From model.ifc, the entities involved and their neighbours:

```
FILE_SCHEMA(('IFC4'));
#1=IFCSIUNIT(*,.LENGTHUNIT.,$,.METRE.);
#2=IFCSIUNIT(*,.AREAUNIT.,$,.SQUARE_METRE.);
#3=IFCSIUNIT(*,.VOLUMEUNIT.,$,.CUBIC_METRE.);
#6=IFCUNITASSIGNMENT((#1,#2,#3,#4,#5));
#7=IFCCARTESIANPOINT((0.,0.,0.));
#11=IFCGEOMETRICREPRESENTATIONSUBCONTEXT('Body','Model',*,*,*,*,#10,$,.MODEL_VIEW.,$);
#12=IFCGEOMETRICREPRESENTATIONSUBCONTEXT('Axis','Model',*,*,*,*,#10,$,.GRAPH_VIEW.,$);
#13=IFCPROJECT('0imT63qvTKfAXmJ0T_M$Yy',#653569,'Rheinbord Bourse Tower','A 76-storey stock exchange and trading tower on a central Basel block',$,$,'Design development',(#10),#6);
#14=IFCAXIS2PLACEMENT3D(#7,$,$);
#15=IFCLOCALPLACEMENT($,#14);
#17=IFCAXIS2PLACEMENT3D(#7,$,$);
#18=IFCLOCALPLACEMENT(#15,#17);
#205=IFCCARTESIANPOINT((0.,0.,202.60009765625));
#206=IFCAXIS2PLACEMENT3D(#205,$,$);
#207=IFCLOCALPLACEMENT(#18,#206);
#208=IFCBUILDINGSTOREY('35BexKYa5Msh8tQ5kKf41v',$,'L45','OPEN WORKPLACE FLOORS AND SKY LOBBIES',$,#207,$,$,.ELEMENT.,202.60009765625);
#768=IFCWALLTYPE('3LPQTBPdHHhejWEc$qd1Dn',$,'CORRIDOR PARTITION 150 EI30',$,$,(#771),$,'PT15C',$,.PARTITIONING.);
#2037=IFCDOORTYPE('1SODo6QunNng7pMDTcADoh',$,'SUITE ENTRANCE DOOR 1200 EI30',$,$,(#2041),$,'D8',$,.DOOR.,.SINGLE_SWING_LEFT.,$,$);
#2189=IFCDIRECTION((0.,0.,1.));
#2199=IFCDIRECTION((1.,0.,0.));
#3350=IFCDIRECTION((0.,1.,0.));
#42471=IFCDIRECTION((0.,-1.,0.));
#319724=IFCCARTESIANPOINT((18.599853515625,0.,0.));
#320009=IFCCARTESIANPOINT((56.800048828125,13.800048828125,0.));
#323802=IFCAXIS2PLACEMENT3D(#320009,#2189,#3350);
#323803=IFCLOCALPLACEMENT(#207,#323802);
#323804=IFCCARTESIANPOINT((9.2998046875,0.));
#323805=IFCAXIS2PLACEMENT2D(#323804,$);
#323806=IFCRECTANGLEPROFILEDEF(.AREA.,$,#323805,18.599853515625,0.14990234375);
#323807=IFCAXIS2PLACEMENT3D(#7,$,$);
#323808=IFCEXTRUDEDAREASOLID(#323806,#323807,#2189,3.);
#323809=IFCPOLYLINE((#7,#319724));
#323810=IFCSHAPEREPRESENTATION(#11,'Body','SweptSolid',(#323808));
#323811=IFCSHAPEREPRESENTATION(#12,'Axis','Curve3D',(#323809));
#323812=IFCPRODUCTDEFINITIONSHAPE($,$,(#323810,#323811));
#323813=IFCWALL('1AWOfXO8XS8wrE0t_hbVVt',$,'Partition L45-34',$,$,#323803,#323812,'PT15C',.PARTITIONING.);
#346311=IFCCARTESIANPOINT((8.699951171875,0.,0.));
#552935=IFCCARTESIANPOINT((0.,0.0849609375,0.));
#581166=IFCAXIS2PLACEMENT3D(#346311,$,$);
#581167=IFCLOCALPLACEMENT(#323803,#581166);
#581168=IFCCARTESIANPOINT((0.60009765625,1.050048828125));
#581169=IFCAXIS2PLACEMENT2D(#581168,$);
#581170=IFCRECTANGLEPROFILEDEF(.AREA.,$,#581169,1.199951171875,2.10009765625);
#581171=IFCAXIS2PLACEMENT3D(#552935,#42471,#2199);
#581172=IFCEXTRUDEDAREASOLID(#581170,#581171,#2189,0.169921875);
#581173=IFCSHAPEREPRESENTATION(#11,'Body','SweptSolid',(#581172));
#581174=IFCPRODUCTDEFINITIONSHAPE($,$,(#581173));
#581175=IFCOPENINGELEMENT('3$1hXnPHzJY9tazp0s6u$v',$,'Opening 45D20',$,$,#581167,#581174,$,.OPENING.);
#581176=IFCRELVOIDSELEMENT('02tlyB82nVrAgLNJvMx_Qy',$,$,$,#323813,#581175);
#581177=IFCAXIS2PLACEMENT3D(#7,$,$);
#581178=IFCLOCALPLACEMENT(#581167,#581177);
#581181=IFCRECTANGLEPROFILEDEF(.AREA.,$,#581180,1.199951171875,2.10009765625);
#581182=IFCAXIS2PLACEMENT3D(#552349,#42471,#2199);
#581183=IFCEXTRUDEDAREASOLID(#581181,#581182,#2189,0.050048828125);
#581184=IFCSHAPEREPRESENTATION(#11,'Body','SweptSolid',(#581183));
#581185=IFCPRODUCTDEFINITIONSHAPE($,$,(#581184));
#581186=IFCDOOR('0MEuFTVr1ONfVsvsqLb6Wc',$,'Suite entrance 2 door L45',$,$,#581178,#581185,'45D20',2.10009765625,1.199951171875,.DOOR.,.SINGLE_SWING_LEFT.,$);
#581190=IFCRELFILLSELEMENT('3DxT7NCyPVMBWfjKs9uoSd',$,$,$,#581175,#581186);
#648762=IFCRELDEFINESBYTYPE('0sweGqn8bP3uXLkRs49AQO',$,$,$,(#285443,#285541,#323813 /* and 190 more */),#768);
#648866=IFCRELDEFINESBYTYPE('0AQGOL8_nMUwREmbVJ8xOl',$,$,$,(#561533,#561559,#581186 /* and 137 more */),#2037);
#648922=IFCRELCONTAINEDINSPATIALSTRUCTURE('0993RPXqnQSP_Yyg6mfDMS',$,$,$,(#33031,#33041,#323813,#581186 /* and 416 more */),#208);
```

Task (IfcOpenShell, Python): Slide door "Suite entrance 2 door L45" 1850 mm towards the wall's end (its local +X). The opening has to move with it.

```python
import ifcopenshell
import ifcopenshell.api.geometry
import ifcopenshell.util.placement
import ifcopenshell.util.unit

model = ifcopenshell.open("model.ifc")
unit_scale = ifcopenshell.util.unit.calculate_unit_scale(model)

door = model.by_guid("0MEuFTVr1ONfVsvsqLb6Wc")
opening = door.FillsVoids[0].RelatingOpeningElement
wall = opening.VoidsElements[0].RelatingBuildingElement

wall_matrix = ifcopenshell.util.placement.get_local_placement(wall.ObjectPlacement)
shift = wall_matrix[:3, 0] * 1.85 / unit_scale
before = ifcopenshell.util.placement.get_local_placement(door.ObjectPlacement)[:3, 3].copy()

# The door is placed relative to its opening, so it follows when the opening moves.
matrix = ifcopenshell.util.placement.get_local_placement(opening.ObjectPlacement)
matrix[:3, 3] += shift
ifcopenshell.api.geometry.edit_object_placement(
    model, product=opening, matrix=matrix, is_si=False, should_transform_children=True
)

after = ifcopenshell.util.placement.get_local_placement(door.ObjectPlacement)[:3, 3]
print("door moved by", (after - before).round(3) + 0.0)

model.write("model_v2.ifc")
```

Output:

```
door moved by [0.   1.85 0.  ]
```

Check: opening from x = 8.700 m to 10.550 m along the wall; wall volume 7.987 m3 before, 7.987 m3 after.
